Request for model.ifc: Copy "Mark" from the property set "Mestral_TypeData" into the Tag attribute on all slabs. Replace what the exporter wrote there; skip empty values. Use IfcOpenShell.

First a look at what the model holds.

```python
import ifcopenshell
import ifcopenshell.util.element

model = ifcopenshell.open("model.ifc")
print(model.schema)
slabs = model.by_type("IfcSlab")
print(len(slabs), "slabs")
for e in slabs[:8]:
    source = ifcopenshell.util.element.get_pset(e, "Mestral_TypeData", "Mark")
    target = e.Tag
    print(e.id(), repr(source), repr(target), sep=" | ")
```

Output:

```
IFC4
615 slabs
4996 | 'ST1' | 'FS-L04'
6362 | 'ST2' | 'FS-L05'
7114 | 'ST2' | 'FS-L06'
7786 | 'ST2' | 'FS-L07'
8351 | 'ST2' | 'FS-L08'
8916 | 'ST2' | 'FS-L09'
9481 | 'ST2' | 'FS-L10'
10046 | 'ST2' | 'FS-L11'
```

```python
import ifcopenshell
import ifcopenshell.util.element

model = ifcopenshell.open("model.ifc")

count = 0
for e in model.by_type("IfcSlab"):
    value = ifcopenshell.util.element.get_pset(e, "Mestral_TypeData", "Mark")
    current = e.Tag
    if not value or not value.strip() or current == value:
        continue
    e.Tag = value
    count += 1

print(count, "slabs updated")

model.write("model_edited.ifc")
```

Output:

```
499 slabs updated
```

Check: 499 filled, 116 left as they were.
